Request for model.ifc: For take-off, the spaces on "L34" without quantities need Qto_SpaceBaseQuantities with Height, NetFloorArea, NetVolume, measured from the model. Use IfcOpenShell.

First a look at what the model holds.

```python
import ifcopenshell
import ifcopenshell.util.element
import ifcopenshell.util.unit

model = ifcopenshell.open("model.ifc")
print(model.schema)
for unit_type in ("LENGTHUNIT", "AREAUNIT", "VOLUMEUNIT"):
    print(unit_type, ifcopenshell.util.unit.calculate_unit_scale(model, unit_type))
storey = next(s for s in model.by_type("IfcBuildingStorey") if s.Name == "L34")
spaces = [e for e in ifcopenshell.util.element.get_decomposition(storey) if e.is_a("IfcSpace")]
for e in sorted(spaces, key=lambda e: e.id()):
    print(e.id(), e.is_a(), e.Name, list(ifcopenshell.util.element.get_psets(e, qtos_only=True)), sep=" | ")
```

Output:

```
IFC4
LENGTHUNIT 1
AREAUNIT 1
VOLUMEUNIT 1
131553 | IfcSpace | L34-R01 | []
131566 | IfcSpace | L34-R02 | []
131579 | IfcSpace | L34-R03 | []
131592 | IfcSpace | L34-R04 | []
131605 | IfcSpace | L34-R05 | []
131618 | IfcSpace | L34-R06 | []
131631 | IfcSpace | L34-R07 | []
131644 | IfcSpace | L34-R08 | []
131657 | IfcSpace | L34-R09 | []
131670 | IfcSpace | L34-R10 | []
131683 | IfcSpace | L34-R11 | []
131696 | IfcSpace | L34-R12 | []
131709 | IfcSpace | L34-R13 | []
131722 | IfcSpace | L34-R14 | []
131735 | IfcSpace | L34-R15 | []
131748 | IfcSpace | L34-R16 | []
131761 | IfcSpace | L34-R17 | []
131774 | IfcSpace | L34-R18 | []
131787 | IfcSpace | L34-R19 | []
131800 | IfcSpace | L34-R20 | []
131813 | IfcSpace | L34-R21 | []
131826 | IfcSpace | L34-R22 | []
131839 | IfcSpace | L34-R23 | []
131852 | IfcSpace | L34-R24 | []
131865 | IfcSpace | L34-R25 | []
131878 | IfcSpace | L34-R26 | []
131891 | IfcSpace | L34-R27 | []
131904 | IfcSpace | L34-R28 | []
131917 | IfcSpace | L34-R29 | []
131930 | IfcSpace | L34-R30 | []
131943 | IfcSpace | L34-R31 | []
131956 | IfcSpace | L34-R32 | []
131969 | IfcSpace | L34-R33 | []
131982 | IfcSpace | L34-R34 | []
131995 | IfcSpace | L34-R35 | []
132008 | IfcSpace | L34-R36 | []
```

```python
import ifcopenshell
import ifcopenshell.api.pset
import ifcopenshell.geom
import ifcopenshell.util.element
import ifcopenshell.util.shape
import ifcopenshell.util.unit

model = ifcopenshell.open("model.ifc")
unit_scale = ifcopenshell.util.unit.calculate_unit_scale(model)
area_scale = ifcopenshell.util.unit.calculate_unit_scale(model, "AREAUNIT")
volume_scale = ifcopenshell.util.unit.calculate_unit_scale(model, "VOLUMEUNIT")
settings = ifcopenshell.geom.settings()

storey = next(s for s in model.by_type("IfcBuildingStorey") if s.Name == "L34")
spaces = [e for e in ifcopenshell.util.element.get_decomposition(storey) if e.is_a("IfcSpace")]

for e in sorted(spaces, key=lambda e: e.id()):
    if ifcopenshell.util.element.get_psets(e, qtos_only=True, should_inherit=False):
        continue
    # Geometry comes back in metres, in the element's own axes.
    shape = ifcopenshell.geom.create_shape(settings, e)
    values = {
        "Height": ifcopenshell.util.shape.get_z(shape.geometry) / unit_scale,
        "NetFloorArea": ifcopenshell.util.shape.get_footprint_area(shape.geometry) / area_scale,
        "NetVolume": ifcopenshell.util.shape.get_volume(shape.geometry) / volume_scale,
    }
    qto = ifcopenshell.api.pset.add_qto(model, product=e, name="Qto_SpaceBaseQuantities")
    ifcopenshell.api.pset.edit_qto(model, qto=qto, properties=values)
    print(e.id(), {k: round(v, 3) for k, v in values.items()})

model.write("model_rev.ifc")
```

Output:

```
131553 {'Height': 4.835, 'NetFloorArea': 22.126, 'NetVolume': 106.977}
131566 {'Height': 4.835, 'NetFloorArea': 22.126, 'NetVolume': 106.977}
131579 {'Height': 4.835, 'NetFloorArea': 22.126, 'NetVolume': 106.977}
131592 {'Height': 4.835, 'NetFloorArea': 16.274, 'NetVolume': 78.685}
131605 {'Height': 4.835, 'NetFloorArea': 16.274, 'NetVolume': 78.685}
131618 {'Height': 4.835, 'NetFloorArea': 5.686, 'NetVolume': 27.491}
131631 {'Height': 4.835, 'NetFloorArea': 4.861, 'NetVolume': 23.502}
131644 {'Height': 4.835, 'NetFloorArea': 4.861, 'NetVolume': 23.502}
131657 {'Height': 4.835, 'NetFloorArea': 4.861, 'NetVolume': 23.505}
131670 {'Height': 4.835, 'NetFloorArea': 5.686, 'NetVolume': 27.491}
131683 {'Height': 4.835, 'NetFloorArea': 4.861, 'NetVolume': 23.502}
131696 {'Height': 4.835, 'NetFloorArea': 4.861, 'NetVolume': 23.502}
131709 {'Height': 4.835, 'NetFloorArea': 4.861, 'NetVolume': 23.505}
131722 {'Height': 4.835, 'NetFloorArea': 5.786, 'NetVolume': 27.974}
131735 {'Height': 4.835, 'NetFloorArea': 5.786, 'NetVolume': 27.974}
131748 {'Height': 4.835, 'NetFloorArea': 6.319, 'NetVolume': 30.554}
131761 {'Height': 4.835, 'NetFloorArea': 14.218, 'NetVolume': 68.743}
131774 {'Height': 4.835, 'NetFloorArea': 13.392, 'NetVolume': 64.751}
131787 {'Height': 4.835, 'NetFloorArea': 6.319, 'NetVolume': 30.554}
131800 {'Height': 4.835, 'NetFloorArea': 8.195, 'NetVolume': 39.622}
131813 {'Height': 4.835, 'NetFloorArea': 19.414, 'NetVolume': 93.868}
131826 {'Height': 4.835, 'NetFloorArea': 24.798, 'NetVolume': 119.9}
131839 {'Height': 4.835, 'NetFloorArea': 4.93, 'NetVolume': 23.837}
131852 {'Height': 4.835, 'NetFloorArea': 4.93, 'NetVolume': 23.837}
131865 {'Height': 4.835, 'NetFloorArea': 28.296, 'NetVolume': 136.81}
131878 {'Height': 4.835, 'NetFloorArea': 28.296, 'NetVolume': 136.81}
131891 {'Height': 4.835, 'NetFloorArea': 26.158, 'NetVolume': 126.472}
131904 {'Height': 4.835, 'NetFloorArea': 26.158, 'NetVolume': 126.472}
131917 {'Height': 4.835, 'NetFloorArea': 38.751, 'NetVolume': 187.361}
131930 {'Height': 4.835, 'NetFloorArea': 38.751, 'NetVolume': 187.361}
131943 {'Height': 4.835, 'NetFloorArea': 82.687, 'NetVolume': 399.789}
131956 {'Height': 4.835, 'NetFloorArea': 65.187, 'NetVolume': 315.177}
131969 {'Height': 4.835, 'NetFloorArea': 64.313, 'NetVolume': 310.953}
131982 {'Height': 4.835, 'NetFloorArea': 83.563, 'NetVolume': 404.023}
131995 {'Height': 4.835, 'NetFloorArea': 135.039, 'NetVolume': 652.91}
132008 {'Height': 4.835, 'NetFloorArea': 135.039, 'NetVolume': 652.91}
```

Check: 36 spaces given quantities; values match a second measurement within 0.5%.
